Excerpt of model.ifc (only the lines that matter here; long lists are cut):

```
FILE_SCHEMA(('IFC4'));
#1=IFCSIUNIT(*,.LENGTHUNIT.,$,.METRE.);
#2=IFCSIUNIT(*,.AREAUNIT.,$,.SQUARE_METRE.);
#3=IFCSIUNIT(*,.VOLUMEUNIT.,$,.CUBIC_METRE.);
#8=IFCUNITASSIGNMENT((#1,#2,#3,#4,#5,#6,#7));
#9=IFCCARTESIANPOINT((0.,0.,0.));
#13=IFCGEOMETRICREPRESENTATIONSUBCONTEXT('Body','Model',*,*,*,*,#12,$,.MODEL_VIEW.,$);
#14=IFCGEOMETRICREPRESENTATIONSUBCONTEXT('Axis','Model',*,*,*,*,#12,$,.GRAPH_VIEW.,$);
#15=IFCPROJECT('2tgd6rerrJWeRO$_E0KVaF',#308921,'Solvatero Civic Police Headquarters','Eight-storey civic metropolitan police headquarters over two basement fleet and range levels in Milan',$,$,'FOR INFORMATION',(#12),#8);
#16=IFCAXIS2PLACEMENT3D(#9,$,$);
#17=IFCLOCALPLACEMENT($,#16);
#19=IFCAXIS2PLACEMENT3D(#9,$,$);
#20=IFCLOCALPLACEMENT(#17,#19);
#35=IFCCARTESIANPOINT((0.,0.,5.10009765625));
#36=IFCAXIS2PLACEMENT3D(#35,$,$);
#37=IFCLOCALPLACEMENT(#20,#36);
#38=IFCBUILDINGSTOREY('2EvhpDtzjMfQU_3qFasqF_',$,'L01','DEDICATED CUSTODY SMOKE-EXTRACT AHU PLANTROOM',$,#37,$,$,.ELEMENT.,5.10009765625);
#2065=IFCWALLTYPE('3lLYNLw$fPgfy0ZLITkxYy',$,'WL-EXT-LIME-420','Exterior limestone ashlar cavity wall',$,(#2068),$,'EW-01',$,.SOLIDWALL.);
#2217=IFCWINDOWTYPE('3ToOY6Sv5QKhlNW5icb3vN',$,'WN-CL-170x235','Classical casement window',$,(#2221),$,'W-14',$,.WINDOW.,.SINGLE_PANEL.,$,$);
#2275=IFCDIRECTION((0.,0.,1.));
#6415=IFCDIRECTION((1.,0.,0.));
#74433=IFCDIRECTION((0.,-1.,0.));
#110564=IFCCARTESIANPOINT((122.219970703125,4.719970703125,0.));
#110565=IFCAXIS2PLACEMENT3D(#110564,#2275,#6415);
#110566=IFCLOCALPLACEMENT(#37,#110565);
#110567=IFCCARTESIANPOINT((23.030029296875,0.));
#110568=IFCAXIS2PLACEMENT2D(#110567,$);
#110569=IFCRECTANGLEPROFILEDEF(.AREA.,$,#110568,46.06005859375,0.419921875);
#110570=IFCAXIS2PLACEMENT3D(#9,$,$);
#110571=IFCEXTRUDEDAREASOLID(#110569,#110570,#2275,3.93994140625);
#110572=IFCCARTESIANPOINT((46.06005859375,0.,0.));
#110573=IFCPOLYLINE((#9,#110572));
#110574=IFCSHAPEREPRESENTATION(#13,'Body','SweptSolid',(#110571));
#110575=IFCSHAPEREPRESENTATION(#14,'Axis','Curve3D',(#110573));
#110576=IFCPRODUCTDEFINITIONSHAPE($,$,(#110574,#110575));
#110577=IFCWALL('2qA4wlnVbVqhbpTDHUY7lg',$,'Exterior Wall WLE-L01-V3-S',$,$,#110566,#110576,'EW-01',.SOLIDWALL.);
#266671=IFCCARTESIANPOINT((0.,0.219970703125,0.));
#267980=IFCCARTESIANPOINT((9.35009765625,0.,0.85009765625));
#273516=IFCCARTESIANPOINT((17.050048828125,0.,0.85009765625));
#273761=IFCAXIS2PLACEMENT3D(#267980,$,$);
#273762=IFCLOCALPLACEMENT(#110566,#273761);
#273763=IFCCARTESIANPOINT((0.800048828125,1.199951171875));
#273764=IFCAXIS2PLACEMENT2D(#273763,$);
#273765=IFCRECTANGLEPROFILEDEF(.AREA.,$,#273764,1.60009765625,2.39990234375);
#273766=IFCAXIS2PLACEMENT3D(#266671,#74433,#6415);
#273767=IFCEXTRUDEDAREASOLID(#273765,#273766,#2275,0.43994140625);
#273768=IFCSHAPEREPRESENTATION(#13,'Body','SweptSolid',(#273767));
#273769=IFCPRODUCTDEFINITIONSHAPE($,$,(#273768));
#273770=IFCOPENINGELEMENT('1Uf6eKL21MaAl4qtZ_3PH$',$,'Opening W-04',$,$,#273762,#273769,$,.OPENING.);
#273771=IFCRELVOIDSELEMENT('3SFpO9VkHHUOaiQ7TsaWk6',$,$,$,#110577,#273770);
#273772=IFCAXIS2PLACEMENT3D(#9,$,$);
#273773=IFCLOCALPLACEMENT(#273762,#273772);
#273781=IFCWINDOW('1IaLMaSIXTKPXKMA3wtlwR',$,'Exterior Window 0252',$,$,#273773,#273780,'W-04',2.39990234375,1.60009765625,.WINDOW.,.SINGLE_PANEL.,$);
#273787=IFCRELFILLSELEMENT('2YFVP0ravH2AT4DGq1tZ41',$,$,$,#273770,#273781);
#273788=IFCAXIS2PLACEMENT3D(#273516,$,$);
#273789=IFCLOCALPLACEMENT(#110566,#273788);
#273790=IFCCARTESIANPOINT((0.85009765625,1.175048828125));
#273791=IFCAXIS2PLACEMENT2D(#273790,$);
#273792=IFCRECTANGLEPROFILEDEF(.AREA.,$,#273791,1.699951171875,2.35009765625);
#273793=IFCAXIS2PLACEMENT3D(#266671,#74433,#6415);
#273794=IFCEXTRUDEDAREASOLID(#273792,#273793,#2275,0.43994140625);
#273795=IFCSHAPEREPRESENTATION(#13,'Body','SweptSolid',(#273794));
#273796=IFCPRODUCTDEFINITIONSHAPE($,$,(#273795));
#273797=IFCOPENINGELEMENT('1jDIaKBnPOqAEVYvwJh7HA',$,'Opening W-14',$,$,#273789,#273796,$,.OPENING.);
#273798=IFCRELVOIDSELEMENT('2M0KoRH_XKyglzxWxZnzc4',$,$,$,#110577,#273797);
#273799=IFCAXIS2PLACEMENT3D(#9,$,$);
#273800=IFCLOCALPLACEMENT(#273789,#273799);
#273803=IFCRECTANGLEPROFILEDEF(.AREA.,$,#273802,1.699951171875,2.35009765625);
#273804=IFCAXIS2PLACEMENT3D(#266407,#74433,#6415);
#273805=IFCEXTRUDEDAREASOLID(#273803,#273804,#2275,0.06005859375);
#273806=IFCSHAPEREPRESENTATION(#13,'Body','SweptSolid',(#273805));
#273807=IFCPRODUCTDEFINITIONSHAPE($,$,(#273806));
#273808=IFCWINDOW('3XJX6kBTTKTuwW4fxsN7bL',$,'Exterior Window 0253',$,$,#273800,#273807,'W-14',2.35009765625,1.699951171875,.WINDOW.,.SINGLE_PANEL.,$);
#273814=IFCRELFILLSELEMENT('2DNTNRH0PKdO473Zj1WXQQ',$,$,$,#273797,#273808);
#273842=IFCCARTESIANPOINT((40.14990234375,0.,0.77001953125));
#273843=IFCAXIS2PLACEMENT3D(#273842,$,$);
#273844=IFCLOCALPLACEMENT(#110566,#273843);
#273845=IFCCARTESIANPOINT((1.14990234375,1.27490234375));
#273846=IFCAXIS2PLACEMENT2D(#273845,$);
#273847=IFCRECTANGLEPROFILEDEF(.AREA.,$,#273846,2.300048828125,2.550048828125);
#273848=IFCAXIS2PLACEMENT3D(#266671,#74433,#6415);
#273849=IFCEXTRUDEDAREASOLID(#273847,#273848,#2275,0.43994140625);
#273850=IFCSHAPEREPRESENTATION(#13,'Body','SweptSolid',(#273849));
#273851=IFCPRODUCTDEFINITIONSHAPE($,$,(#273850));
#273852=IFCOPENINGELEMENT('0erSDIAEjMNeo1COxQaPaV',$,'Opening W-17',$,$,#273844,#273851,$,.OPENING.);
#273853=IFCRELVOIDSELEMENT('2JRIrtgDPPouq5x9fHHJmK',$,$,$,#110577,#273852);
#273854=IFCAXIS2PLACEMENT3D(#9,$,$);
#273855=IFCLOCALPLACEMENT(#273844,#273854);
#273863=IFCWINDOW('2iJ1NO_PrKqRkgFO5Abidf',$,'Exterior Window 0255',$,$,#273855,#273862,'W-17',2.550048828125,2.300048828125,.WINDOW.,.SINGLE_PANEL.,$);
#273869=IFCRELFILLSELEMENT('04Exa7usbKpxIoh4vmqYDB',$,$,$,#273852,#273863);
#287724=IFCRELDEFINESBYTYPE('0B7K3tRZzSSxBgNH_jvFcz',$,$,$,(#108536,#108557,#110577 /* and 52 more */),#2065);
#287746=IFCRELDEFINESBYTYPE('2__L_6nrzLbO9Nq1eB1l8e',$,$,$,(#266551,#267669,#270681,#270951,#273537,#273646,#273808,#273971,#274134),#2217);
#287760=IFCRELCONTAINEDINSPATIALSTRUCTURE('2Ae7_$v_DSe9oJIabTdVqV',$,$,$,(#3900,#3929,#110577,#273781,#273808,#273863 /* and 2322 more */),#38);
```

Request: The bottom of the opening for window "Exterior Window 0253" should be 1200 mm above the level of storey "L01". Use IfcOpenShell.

```python
import numpy as np
import ifcopenshell
import ifcopenshell.api.geometry
import ifcopenshell.geom
import ifcopenshell.util.element
import ifcopenshell.util.placement
import ifcopenshell.util.shape
import ifcopenshell.util.unit

model = ifcopenshell.open("model.ifc")
unit_scale = ifcopenshell.util.unit.calculate_unit_scale(model)

window = model.by_id(273808)
opening = window.FillsVoids[0].RelatingOpeningElement
storey = ifcopenshell.util.element.get_container(window, ifc_class="IfcBuildingStorey")
level = ifcopenshell.util.placement.get_local_placement(storey.ObjectPlacement)[2, 3]

# The opening's origin need not be at the sill, so measure its lowest point.
shape = ifcopenshell.geom.create_shape(ifcopenshell.geom.settings(), opening)
bottom = ifcopenshell.util.shape.get_shape_bottom_elevation(shape, shape.geometry) / unit_scale
dz = level + 1.2 - bottom

shift = np.array([0.0, 0.0, dz])
# The window is placed relative to its opening, so it follows when the opening moves.
matrix = ifcopenshell.util.placement.get_local_placement(opening.ObjectPlacement)
matrix[:3, 3] += shift
ifcopenshell.api.geometry.edit_object_placement(
    model, product=opening, matrix=matrix, is_si=False, should_transform_children=True
)

print(f"moved by {dz * unit_scale:+.3f} m")

model.write("model_v2.ifc")
```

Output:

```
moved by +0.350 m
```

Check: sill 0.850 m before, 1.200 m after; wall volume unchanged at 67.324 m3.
